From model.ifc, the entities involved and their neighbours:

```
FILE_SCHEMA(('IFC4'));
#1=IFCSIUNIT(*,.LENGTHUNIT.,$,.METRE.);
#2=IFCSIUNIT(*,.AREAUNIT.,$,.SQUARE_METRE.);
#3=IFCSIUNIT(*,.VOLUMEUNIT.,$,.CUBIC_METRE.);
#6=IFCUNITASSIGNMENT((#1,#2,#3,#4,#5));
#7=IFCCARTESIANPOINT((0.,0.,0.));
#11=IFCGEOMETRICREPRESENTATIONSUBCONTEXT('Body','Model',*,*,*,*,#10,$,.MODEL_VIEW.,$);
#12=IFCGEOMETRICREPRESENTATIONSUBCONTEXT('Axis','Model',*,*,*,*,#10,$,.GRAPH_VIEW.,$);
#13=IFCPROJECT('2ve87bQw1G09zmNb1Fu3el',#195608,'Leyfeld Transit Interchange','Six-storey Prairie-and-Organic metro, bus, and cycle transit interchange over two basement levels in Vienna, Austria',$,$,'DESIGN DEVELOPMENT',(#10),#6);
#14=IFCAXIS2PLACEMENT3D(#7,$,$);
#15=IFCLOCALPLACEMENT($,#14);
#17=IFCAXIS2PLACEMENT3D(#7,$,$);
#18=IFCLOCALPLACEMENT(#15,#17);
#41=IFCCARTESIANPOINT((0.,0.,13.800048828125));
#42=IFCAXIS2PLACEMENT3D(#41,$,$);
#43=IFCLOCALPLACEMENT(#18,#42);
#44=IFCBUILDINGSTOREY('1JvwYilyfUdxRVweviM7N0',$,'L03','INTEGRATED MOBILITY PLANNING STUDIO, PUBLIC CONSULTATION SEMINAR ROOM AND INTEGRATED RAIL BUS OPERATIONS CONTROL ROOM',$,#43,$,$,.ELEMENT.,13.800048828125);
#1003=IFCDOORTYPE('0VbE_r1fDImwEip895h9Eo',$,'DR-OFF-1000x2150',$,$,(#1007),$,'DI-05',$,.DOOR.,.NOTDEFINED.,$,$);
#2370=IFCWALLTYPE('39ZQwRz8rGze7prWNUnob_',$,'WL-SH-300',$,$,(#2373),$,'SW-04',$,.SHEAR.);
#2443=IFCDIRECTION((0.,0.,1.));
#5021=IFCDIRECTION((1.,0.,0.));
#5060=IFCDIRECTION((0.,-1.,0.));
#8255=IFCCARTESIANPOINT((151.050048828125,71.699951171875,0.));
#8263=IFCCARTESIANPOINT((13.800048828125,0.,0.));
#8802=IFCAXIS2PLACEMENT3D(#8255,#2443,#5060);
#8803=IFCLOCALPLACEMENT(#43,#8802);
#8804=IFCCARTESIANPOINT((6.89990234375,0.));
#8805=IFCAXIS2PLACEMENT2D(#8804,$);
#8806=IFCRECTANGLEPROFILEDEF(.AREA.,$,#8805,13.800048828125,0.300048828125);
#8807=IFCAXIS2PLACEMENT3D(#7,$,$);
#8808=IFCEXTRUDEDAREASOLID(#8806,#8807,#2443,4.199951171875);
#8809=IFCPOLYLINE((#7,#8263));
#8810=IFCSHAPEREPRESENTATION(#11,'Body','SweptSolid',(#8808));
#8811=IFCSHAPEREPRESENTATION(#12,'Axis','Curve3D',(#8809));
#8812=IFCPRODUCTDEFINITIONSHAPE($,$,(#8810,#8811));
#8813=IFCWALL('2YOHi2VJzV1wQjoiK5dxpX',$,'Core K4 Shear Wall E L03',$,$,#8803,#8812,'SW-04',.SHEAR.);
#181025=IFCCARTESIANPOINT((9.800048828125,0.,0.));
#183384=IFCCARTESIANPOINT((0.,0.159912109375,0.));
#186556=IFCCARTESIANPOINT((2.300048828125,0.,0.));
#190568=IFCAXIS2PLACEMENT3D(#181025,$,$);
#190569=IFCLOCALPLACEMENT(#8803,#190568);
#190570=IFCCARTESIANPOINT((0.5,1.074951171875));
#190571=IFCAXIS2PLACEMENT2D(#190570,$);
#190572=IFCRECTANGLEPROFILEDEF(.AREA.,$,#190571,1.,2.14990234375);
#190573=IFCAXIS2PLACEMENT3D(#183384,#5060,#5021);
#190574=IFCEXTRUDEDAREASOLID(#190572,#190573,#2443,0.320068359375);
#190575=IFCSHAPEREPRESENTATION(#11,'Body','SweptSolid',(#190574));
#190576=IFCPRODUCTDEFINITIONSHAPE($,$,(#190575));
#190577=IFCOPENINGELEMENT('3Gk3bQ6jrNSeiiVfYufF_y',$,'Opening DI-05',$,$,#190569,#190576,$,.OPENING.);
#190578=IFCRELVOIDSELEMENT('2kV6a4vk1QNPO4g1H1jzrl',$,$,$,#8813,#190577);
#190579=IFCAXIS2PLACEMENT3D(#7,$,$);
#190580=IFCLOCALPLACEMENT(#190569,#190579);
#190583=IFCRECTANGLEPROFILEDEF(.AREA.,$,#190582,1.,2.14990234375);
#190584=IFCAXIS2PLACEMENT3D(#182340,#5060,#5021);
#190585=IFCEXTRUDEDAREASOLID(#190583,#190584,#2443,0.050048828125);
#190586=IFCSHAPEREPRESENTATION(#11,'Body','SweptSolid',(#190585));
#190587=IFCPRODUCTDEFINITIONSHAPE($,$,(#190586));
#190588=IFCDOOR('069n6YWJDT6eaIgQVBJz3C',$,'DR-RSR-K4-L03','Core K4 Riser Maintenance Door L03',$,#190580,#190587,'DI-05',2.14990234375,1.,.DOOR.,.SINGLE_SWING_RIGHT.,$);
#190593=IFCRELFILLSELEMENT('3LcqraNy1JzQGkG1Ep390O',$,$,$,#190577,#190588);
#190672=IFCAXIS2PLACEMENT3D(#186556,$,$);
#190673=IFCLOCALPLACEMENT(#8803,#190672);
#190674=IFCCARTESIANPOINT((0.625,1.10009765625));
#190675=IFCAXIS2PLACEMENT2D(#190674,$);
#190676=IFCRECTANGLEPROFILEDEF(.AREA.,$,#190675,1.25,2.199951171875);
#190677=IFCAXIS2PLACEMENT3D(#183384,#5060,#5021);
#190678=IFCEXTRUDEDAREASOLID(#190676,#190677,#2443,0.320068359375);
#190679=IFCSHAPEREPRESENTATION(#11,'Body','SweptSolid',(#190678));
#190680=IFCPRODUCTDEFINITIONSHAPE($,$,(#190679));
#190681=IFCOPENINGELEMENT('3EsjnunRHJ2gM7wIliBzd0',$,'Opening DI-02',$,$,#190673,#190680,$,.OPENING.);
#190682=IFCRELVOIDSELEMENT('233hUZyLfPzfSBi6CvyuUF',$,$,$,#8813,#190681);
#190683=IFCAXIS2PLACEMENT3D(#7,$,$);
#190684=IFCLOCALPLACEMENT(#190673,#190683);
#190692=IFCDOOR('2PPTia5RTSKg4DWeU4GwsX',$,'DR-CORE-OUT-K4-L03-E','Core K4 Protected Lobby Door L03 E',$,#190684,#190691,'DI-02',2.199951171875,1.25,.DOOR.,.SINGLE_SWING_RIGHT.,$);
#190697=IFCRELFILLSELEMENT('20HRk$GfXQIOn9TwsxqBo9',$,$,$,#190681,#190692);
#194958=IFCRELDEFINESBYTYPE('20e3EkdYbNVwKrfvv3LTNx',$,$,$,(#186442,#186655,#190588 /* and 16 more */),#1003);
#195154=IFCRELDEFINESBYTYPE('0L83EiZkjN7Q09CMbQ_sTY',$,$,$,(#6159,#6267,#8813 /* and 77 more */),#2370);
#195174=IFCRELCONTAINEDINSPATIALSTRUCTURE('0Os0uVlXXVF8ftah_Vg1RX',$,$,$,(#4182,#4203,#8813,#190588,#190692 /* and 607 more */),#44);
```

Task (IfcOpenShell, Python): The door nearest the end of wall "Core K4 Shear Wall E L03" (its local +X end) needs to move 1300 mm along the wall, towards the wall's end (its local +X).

```python
import ifcopenshell
import ifcopenshell.api.geometry
import ifcopenshell.util.placement
import ifcopenshell.util.unit

model = ifcopenshell.open("model.ifc")
unit_scale = ifcopenshell.util.unit.calculate_unit_scale(model)

door = model.by_guid("069n6YWJDT6eaIgQVBJz3C")
opening = door.FillsVoids[0].RelatingOpeningElement
wall = opening.VoidsElements[0].RelatingBuildingElement

wall_matrix = ifcopenshell.util.placement.get_local_placement(wall.ObjectPlacement)
shift = wall_matrix[:3, 0] * 1.3 / unit_scale
before = ifcopenshell.util.placement.get_local_placement(door.ObjectPlacement)[:3, 3].copy()

# The door is placed relative to its opening, so it follows when the opening moves.
matrix = ifcopenshell.util.placement.get_local_placement(opening.ObjectPlacement)
matrix[:3, 3] += shift
ifcopenshell.api.geometry.edit_object_placement(
    model, product=opening, matrix=matrix, is_si=False, should_transform_children=True
)

after = ifcopenshell.util.placement.get_local_placement(door.ObjectPlacement)[:3, 3]
print("door moved by", (after - before).round(3) + 0.0)

model.write("model_edited.ifc")
```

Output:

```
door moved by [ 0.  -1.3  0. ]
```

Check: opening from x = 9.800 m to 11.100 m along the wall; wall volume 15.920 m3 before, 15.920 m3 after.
